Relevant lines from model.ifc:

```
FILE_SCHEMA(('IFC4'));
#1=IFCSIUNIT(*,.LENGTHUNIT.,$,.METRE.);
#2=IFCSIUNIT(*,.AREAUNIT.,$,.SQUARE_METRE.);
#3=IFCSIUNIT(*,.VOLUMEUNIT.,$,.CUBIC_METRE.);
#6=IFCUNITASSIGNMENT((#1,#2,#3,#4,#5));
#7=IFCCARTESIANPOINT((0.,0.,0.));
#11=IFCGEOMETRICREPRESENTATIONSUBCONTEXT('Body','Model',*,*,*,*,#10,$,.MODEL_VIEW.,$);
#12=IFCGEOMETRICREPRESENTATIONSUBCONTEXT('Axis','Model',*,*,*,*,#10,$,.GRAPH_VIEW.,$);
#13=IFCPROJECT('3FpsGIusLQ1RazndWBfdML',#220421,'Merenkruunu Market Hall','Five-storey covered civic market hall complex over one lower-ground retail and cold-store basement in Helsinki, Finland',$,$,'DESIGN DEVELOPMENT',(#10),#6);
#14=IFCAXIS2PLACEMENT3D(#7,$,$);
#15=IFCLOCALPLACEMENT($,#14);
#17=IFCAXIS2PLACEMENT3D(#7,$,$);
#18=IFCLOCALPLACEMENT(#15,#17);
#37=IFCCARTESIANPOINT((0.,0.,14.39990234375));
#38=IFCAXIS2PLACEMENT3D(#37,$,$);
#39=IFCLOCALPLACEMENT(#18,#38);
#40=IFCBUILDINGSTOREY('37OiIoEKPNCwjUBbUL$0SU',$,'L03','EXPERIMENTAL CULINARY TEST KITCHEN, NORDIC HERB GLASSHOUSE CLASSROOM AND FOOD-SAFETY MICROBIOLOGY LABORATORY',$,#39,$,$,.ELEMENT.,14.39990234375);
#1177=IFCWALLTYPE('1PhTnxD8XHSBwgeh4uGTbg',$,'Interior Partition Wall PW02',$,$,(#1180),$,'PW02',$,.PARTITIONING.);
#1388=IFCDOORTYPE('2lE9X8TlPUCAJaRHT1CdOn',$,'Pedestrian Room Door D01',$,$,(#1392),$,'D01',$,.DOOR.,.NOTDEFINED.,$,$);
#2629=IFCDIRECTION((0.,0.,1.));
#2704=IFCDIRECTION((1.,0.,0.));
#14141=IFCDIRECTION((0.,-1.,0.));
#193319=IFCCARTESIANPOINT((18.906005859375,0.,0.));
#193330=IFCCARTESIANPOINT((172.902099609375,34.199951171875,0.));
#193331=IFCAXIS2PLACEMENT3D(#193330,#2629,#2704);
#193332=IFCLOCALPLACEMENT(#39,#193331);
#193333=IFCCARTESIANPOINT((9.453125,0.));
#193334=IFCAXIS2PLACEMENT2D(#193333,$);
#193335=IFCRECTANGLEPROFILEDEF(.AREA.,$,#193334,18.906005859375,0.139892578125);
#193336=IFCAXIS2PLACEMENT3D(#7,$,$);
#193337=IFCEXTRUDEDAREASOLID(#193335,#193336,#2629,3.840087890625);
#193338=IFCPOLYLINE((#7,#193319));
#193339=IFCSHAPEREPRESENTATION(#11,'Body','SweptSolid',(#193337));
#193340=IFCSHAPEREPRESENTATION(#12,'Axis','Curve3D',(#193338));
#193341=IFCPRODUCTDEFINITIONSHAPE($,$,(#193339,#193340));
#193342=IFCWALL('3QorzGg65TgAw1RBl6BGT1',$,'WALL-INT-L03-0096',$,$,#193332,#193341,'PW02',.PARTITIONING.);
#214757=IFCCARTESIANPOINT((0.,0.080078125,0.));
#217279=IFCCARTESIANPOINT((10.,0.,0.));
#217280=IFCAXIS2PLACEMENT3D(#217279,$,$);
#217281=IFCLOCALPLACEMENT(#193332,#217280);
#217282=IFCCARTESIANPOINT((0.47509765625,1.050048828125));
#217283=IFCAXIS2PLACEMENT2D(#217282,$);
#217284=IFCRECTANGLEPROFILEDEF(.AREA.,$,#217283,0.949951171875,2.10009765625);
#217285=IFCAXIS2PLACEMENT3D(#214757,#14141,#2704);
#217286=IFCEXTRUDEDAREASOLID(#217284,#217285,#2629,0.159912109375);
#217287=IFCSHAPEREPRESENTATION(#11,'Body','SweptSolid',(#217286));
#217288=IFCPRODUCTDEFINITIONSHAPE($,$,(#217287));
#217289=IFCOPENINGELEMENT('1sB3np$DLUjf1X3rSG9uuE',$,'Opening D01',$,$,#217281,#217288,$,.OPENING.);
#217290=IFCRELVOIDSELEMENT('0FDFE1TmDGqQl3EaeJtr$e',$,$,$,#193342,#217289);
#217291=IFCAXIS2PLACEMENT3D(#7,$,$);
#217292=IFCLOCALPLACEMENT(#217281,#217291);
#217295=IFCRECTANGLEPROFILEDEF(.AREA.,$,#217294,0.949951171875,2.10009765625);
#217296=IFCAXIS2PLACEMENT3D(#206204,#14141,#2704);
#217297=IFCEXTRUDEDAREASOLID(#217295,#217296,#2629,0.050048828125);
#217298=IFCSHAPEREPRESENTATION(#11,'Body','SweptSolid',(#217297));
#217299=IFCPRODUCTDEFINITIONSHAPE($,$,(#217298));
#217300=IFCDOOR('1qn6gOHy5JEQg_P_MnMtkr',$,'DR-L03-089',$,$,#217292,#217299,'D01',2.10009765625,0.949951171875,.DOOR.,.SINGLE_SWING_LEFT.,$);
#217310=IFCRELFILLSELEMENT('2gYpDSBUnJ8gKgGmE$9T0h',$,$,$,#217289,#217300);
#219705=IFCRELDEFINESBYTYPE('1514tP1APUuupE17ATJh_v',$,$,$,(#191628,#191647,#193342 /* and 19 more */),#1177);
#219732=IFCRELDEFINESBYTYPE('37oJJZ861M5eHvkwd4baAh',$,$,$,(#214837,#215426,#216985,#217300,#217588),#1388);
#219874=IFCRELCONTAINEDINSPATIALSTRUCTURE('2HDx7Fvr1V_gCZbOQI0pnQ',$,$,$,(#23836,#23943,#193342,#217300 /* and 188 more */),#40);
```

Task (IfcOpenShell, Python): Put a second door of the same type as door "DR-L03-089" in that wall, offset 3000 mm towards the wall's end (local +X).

```python
import ifcopenshell
import ifcopenshell.api.feature
import ifcopenshell.api.geometry
import ifcopenshell.api.root
import ifcopenshell.geom
import ifcopenshell.util.element
import ifcopenshell.util.placement
import ifcopenshell.util.shape
import ifcopenshell.util.unit

model = ifcopenshell.open("model.ifc")
unit_scale = ifcopenshell.util.unit.calculate_unit_scale(model)
settings = ifcopenshell.geom.settings()


def volume(element):
    """Net volume in cubic metres, openings subtracted."""
    shape = ifcopenshell.geom.create_shape(settings, element)
    return ifcopenshell.util.shape.get_volume(shape.geometry)


door = model.by_guid("1qn6gOHy5JEQg_P_MnMtkr")
opening = door.FillsVoids[0].RelatingOpeningElement
wall = opening.VoidsElements[0].RelatingBuildingElement
before = volume(wall)
shift = ifcopenshell.util.placement.get_local_placement(wall.ObjectPlacement)[:3, 0] * 3 / unit_scale

# copy_class copies the void relationship, type, container and properties, but no geometry.
new_opening = ifcopenshell.api.root.copy_class(model, product=opening)
new_opening.Representation = ifcopenshell.util.element.copy_deep(
    model, opening.Representation, exclude=["IfcGeometricRepresentationContext", "IfcRepresentationMap"]
)
new_door = ifcopenshell.api.root.copy_class(model, product=door)
new_door.Representation = ifcopenshell.util.element.copy_deep(
    model, door.Representation, exclude=["IfcGeometricRepresentationContext", "IfcRepresentationMap"]
)
new_door.Tag = None
ifcopenshell.api.feature.add_filling(model, opening=new_opening, element=new_door)

for old, new in ((opening, new_opening), (door, new_door)):
    matrix = ifcopenshell.util.placement.get_local_placement(old.ObjectPlacement)
    matrix[:3, 3] += shift
    ifcopenshell.api.geometry.edit_object_placement(model, product=new, matrix=matrix, is_si=False)

after = volume(wall)

print(f"wall volume {before:.3f} -> {after:.3f} m3")

model.write("model-out.ifc")
```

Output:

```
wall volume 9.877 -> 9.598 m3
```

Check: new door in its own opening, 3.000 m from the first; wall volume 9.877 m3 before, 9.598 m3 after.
